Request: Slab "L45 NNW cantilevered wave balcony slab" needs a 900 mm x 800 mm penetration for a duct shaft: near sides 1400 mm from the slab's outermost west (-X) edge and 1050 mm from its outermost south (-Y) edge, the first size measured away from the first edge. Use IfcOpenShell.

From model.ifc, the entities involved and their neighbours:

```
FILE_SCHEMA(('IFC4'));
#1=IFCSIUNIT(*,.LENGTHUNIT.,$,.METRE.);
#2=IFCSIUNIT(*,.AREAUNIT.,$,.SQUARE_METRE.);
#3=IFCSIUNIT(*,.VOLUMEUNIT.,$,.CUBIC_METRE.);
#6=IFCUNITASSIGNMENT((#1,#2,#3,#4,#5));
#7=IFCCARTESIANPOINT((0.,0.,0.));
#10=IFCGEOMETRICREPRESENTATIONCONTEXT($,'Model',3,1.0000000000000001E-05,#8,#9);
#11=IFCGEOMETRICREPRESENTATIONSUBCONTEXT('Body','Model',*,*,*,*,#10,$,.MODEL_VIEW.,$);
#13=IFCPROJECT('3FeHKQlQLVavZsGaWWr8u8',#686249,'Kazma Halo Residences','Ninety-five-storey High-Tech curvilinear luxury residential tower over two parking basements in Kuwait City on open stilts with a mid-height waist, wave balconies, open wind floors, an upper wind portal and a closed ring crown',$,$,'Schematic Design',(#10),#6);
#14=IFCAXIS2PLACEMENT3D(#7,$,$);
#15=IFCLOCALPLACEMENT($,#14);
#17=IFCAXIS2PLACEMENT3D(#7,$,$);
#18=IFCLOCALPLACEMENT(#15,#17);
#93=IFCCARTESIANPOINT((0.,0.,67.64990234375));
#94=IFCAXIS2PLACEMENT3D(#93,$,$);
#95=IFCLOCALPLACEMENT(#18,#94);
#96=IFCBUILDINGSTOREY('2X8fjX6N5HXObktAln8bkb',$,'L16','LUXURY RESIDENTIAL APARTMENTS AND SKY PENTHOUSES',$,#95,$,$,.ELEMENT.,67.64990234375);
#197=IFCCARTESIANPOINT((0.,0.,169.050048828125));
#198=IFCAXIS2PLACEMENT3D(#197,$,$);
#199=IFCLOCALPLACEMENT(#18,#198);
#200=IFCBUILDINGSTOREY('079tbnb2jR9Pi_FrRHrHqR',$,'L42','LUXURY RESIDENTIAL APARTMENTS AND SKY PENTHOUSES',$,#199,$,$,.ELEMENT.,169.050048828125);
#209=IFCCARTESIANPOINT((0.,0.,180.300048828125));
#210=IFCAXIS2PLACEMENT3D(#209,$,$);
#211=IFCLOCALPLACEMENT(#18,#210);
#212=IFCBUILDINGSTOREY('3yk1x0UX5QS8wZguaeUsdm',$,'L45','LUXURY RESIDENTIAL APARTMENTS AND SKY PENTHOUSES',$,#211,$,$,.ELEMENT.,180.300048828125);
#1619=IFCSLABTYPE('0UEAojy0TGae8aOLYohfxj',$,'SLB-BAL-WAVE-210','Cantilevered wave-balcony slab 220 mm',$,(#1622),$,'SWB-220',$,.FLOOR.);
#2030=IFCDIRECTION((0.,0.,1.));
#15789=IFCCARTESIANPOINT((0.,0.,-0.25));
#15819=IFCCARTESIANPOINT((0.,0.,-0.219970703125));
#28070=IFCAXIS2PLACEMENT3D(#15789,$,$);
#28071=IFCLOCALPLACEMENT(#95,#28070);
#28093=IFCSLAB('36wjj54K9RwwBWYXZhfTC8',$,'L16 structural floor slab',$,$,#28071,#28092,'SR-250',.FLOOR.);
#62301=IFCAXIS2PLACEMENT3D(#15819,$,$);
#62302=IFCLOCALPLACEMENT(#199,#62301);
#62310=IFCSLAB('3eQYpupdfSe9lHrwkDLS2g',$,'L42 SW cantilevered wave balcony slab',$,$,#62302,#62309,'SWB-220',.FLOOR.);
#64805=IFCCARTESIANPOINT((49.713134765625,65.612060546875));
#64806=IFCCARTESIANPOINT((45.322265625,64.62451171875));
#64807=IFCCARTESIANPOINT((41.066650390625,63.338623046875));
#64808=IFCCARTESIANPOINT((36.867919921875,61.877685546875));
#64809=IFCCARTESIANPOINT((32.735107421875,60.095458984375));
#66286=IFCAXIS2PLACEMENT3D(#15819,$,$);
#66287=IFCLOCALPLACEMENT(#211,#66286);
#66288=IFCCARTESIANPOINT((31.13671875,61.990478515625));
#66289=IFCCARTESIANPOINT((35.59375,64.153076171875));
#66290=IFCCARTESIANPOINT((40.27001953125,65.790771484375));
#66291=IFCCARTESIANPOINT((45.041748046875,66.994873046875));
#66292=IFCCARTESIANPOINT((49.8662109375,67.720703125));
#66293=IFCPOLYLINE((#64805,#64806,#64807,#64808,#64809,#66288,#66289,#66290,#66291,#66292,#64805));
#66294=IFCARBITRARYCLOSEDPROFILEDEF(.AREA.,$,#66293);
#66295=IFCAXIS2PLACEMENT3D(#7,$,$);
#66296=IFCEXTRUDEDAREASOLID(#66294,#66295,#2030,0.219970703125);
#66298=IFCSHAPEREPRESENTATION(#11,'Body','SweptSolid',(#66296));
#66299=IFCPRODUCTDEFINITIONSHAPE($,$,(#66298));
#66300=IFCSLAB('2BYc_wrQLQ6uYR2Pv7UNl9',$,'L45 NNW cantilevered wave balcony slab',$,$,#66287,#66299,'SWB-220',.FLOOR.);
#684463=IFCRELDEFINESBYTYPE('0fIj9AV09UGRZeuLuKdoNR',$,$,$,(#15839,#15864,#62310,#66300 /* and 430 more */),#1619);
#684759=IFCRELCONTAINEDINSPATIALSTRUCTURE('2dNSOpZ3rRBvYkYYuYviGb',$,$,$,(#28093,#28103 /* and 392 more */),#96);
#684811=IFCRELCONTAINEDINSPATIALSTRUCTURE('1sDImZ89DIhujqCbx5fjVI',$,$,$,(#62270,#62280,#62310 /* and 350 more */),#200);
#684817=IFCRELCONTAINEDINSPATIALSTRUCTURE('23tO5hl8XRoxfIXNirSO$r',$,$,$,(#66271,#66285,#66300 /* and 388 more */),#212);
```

```python
import numpy as np
import ifcopenshell
import ifcopenshell.api.feature
import ifcopenshell.api.geometry
import ifcopenshell.api.root
import ifcopenshell.geom
import ifcopenshell.util.placement
import ifcopenshell.util.representation
import ifcopenshell.util.shape
import ifcopenshell.util.unit

model = ifcopenshell.open("model.ifc")
unit_scale = ifcopenshell.util.unit.calculate_unit_scale(model)
settings = ifcopenshell.geom.settings()


def volume(element):
    """Net volume in cubic metres, openings subtracted."""
    shape = ifcopenshell.geom.create_shape(settings, element)
    return ifcopenshell.util.shape.get_volume(shape.geometry)


slab = model.by_guid("2BYc_wrQLQ6uYR2Pv7UNl9")
before = volume(slab)

# Extent in the slab's own axes, in metres. The edges named are its -X and -Y sides.
slab_shape = ifcopenshell.geom.create_shape(settings, slab)
vertices = ifcopenshell.util.shape.get_vertices(slab_shape.geometry)
x_min, y_min, bottom = vertices.min(axis=0)
top = vertices[:, 2].max()

opening = ifcopenshell.api.root.create_entity(model, ifc_class="IfcOpeningElement", name="Duct shaft opening", predefined_type="OPENING")
context = ifcopenshell.util.representation.get_context(model, "Model", "Body", "MODEL_VIEW")
width, depth = 0.9, 0.8
outline = [(0.0, 0.0), (width, 0.0), (width, depth), (0.0, depth), (0.0, 0.0)]
# Overshoot both faces by 50 mm so the cut is clean.
shape = ifcopenshell.api.geometry.add_slab_representation(
    model, context=context, depth=top - bottom + 0.1, polyline=outline
)
ifcopenshell.api.geometry.assign_representation(model, product=opening, representation=shape)

matrix = ifcopenshell.util.placement.get_local_placement(slab.ObjectPlacement)
matrix[:, 3] = matrix @ np.append(np.array([x_min + 1.4, y_min + 1.05, bottom - 0.05]) / unit_scale, 1.0)
ifcopenshell.api.geometry.edit_object_placement(model, product=opening, matrix=matrix, is_si=False)
ifcopenshell.api.feature.add_feature(model, feature=opening, element=slab)

after = volume(slab)

print(f"slab volume {before:.3f} -> {after:.3f} m3")

model.write("model_edited.ifc")
```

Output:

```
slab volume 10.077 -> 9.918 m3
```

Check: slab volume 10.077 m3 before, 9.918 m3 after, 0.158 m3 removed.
